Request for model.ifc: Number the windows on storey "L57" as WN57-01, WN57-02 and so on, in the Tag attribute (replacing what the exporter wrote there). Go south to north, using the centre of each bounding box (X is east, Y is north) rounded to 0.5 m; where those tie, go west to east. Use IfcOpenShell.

First a look at what the model holds.

```python
import ifcopenshell
import ifcopenshell.util.element
import ifcopenshell.util.placement

model = ifcopenshell.open("model.ifc")
print(model.schema)
storey = next(s for s in model.by_type("IfcBuildingStorey") if s.Name == "L57")
windows = [e for e in ifcopenshell.util.element.get_decomposition(storey) if e.is_a("IfcWindow")]
for e in sorted(windows, key=lambda e: e.id()):
    origin = ifcopenshell.util.placement.get_local_placement(e.ObjectPlacement)[:3, 3]
    print(e.id(), e.Tag, e.Name, origin.round(2) + 0.0, sep=" | ")
```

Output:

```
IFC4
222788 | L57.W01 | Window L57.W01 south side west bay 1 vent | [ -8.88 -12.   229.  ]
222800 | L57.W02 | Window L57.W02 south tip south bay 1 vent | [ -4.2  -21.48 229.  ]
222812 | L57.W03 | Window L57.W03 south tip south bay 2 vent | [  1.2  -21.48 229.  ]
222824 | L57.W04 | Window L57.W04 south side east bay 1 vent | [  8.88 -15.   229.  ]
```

```python
import ifcopenshell
import ifcopenshell.geom
import ifcopenshell.util.element
import ifcopenshell.util.shape

model = ifcopenshell.open("model.ifc")
settings = ifcopenshell.geom.settings()
settings.set("use-world-coords", True)


def centre(element):
    shape = ifcopenshell.geom.create_shape(settings, element)
    return ifcopenshell.util.shape.get_bbox_centroid(shape.geometry)


storey = next(s for s in model.by_type("IfcBuildingStorey") if s.Name == "L57")
windows = [e for e in ifcopenshell.util.element.get_decomposition(storey) if e.is_a("IfcWindow")]

# Insertion points can sit at a corner or the storey origin, so sort by the geometry (in metres).
centres = {e: centre(e) for e in windows}
windows.sort(key=lambda e: (round(centres[e][1] / 0.5), centres[e][0]))

for i, e in enumerate(windows, start=1):
    number = f"WN57-{i:02d}"
    e.Tag = number
    print(e.id(), number)

model.write("model_updated.ifc")
```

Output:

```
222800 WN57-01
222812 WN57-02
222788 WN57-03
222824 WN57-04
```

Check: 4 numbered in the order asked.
